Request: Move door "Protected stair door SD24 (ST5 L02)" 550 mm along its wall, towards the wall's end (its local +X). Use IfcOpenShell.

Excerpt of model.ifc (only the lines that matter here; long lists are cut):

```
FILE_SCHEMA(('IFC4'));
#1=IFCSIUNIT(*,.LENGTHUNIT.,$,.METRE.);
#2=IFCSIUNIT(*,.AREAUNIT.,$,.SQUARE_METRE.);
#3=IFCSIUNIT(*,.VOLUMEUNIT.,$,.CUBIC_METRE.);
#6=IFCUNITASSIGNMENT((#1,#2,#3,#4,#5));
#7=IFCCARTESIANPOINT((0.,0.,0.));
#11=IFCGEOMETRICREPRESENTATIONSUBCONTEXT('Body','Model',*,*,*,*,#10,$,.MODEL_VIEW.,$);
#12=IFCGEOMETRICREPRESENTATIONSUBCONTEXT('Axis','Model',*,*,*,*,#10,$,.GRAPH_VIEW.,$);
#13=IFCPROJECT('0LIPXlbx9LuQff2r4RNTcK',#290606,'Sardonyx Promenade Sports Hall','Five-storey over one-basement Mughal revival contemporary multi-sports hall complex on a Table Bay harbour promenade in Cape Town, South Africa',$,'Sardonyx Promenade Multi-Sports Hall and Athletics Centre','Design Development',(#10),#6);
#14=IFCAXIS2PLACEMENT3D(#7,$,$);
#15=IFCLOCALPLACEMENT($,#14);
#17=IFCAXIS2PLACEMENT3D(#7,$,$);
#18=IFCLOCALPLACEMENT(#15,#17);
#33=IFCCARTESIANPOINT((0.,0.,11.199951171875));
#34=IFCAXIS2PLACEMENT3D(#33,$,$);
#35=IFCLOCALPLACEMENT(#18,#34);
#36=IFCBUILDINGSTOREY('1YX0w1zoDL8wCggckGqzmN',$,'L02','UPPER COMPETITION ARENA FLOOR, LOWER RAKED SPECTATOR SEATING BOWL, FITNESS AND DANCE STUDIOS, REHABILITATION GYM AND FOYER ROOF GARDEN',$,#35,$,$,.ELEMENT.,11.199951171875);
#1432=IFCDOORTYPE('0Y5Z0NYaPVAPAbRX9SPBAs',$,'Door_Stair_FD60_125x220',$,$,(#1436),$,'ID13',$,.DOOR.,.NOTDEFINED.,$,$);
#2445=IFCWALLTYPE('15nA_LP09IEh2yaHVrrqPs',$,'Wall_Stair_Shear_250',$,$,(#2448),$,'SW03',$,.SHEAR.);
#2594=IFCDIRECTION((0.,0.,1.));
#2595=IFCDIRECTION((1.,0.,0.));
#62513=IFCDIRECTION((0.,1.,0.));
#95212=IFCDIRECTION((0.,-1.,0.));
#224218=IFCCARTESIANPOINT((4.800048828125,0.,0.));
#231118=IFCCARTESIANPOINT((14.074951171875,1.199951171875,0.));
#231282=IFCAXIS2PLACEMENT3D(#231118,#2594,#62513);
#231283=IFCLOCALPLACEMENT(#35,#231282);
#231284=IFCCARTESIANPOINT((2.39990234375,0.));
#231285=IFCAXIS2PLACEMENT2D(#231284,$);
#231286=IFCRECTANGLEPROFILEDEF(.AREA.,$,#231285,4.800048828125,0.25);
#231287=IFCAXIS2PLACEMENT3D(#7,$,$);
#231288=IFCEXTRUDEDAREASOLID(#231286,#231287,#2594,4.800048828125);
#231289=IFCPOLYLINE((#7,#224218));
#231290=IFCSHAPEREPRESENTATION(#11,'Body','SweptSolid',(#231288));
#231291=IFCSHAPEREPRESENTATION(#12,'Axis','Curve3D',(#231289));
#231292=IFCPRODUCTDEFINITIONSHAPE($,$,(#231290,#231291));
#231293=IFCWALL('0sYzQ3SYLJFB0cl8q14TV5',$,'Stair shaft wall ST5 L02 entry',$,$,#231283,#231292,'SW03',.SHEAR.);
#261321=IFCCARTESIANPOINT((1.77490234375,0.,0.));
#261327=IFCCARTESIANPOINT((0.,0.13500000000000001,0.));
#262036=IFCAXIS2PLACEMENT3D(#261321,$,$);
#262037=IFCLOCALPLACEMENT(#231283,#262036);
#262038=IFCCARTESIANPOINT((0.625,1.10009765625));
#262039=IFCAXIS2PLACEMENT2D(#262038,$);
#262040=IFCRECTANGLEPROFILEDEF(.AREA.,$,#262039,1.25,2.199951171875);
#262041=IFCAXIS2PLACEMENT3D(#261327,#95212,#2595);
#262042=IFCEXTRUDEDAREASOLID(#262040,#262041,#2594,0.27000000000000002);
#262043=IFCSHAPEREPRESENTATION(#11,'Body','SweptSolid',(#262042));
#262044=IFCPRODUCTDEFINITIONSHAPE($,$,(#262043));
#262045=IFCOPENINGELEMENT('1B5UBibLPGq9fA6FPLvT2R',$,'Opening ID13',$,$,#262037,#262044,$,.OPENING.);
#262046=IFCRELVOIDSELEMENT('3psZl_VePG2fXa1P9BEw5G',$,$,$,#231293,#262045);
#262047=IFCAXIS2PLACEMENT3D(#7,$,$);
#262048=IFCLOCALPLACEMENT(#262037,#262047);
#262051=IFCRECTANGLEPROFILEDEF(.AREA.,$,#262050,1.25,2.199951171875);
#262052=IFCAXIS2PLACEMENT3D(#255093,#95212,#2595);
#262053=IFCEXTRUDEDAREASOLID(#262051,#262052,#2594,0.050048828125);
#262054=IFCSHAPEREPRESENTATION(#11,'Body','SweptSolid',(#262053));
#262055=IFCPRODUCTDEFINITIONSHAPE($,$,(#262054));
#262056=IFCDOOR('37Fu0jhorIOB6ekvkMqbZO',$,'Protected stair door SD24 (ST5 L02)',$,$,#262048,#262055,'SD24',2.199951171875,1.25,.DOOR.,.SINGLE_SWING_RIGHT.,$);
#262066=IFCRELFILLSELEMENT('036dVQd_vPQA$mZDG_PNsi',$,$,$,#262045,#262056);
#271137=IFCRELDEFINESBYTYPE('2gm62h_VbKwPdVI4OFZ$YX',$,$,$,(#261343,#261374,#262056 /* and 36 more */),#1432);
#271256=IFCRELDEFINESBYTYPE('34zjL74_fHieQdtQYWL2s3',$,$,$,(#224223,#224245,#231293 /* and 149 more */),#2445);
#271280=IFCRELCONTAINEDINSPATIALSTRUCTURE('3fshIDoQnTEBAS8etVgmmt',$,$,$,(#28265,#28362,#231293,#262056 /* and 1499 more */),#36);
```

```python
import ifcopenshell
import ifcopenshell.api.geometry
import ifcopenshell.util.placement
import ifcopenshell.util.unit

model = ifcopenshell.open("model.ifc")
unit_scale = ifcopenshell.util.unit.calculate_unit_scale(model)

door = model.by_guid("37Fu0jhorIOB6ekvkMqbZO")
opening = door.FillsVoids[0].RelatingOpeningElement
wall = opening.VoidsElements[0].RelatingBuildingElement

wall_matrix = ifcopenshell.util.placement.get_local_placement(wall.ObjectPlacement)
shift = wall_matrix[:3, 0] * 0.55 / unit_scale
before = ifcopenshell.util.placement.get_local_placement(door.ObjectPlacement)[:3, 3].copy()

# The door is placed relative to its opening, so it follows when the opening moves.
matrix = ifcopenshell.util.placement.get_local_placement(opening.ObjectPlacement)
matrix[:3, 3] += shift
ifcopenshell.api.geometry.edit_object_placement(
    model, product=opening, matrix=matrix, is_si=False, should_transform_children=True
)

after = ifcopenshell.util.placement.get_local_placement(door.ObjectPlacement)[:3, 3]
print("door moved by", (after - before).round(3) + 0.0)

model.write("model_edited.ifc")
```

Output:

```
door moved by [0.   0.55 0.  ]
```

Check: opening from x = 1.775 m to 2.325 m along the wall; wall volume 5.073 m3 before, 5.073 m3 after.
